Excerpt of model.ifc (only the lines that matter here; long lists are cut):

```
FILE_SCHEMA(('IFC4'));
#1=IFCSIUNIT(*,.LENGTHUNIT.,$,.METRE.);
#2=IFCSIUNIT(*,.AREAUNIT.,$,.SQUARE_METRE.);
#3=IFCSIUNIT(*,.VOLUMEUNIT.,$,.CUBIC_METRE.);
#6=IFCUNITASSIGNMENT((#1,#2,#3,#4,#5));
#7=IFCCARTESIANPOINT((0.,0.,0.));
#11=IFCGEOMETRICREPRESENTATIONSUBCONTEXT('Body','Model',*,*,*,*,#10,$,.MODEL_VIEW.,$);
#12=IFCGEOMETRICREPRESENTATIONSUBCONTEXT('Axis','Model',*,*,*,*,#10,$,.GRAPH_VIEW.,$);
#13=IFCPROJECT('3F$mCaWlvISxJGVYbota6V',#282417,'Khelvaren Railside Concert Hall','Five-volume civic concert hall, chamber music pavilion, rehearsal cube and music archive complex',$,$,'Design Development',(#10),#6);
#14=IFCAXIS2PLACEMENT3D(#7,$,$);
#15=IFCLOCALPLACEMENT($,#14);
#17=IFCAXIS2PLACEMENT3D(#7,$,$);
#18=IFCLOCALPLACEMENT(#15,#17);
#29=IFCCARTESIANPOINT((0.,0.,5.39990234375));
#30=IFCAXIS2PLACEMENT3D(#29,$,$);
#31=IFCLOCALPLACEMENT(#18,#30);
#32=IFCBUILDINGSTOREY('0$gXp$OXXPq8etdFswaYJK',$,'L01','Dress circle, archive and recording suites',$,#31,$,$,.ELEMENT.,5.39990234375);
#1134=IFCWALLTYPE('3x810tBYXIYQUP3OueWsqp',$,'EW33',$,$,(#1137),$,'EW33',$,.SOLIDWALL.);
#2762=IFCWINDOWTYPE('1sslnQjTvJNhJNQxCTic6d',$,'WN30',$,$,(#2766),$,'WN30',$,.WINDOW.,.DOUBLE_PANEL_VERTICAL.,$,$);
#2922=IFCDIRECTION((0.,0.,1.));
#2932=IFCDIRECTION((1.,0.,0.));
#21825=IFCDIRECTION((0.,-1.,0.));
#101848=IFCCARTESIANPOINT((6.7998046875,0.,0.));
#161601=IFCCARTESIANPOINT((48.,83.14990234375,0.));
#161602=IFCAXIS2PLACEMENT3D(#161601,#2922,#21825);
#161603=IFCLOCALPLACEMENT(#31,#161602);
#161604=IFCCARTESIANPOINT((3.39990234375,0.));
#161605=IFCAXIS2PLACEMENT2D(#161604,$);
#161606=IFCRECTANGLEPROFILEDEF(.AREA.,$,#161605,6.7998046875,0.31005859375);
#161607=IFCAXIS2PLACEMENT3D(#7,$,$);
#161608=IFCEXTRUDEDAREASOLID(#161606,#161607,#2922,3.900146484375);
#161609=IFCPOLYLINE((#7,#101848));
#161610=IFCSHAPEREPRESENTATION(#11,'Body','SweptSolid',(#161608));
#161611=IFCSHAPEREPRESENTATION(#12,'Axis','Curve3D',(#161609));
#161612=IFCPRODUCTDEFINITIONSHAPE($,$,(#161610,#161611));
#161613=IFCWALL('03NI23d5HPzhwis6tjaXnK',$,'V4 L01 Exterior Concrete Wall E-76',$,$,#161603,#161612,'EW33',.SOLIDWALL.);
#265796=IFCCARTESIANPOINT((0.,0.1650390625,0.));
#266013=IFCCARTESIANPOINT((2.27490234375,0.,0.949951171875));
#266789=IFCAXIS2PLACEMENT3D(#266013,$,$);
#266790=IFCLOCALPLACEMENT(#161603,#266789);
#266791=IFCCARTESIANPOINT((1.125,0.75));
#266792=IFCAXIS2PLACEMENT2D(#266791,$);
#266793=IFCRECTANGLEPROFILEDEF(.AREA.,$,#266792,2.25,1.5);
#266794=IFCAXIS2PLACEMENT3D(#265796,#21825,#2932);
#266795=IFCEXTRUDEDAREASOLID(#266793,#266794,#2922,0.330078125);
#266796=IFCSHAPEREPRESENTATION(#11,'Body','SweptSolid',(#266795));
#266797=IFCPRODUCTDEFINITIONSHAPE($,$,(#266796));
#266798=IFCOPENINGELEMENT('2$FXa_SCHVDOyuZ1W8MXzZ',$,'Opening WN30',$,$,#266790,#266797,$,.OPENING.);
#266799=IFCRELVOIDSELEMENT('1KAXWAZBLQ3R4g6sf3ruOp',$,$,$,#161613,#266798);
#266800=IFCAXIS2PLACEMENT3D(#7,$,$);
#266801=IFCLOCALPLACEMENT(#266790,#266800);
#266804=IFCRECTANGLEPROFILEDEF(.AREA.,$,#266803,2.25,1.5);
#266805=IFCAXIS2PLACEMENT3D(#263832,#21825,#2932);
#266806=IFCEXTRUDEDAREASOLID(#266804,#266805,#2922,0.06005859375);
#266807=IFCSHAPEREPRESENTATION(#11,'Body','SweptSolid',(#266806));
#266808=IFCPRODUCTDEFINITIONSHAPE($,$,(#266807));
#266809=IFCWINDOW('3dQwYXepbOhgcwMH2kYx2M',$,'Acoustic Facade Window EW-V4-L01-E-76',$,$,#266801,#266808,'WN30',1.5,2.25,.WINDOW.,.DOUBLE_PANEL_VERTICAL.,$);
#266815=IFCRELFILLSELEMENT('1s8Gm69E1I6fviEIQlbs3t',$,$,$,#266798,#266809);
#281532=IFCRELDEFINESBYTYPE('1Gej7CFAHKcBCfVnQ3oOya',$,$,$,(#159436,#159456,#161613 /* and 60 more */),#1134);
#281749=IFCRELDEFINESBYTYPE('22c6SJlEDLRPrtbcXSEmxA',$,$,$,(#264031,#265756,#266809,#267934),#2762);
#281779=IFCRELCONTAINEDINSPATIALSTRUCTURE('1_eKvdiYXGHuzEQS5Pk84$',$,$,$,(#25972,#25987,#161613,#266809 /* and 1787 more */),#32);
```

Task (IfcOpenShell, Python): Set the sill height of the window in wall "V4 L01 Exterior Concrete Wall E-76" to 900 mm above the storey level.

```python
import numpy as np
import ifcopenshell
import ifcopenshell.api.geometry
import ifcopenshell.geom
import ifcopenshell.util.element
import ifcopenshell.util.placement
import ifcopenshell.util.shape
import ifcopenshell.util.unit

model = ifcopenshell.open("model.ifc")
unit_scale = ifcopenshell.util.unit.calculate_unit_scale(model)

window = model.by_guid("3dQwYXepbOhgcwMH2kYx2M")
opening = window.FillsVoids[0].RelatingOpeningElement
storey = ifcopenshell.util.element.get_container(window, ifc_class="IfcBuildingStorey")
level = ifcopenshell.util.placement.get_local_placement(storey.ObjectPlacement)[2, 3]

# The opening's origin need not be at the sill, so measure its lowest point.
shape = ifcopenshell.geom.create_shape(ifcopenshell.geom.settings(), opening)
bottom = ifcopenshell.util.shape.get_shape_bottom_elevation(shape, shape.geometry) / unit_scale
dz = level + 0.9 - bottom

shift = np.array([0.0, 0.0, dz])
# The window is placed relative to its opening, so it follows when the opening moves.
matrix = ifcopenshell.util.placement.get_local_placement(opening.ObjectPlacement)
matrix[:3, 3] += shift
ifcopenshell.api.geometry.edit_object_placement(
    model, product=opening, matrix=matrix, is_si=False, should_transform_children=True
)

print(f"moved by {dz * unit_scale:+.3f} m")

model.write("model_updated.ifc")
```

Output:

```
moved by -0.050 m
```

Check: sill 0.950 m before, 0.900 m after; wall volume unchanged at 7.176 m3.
